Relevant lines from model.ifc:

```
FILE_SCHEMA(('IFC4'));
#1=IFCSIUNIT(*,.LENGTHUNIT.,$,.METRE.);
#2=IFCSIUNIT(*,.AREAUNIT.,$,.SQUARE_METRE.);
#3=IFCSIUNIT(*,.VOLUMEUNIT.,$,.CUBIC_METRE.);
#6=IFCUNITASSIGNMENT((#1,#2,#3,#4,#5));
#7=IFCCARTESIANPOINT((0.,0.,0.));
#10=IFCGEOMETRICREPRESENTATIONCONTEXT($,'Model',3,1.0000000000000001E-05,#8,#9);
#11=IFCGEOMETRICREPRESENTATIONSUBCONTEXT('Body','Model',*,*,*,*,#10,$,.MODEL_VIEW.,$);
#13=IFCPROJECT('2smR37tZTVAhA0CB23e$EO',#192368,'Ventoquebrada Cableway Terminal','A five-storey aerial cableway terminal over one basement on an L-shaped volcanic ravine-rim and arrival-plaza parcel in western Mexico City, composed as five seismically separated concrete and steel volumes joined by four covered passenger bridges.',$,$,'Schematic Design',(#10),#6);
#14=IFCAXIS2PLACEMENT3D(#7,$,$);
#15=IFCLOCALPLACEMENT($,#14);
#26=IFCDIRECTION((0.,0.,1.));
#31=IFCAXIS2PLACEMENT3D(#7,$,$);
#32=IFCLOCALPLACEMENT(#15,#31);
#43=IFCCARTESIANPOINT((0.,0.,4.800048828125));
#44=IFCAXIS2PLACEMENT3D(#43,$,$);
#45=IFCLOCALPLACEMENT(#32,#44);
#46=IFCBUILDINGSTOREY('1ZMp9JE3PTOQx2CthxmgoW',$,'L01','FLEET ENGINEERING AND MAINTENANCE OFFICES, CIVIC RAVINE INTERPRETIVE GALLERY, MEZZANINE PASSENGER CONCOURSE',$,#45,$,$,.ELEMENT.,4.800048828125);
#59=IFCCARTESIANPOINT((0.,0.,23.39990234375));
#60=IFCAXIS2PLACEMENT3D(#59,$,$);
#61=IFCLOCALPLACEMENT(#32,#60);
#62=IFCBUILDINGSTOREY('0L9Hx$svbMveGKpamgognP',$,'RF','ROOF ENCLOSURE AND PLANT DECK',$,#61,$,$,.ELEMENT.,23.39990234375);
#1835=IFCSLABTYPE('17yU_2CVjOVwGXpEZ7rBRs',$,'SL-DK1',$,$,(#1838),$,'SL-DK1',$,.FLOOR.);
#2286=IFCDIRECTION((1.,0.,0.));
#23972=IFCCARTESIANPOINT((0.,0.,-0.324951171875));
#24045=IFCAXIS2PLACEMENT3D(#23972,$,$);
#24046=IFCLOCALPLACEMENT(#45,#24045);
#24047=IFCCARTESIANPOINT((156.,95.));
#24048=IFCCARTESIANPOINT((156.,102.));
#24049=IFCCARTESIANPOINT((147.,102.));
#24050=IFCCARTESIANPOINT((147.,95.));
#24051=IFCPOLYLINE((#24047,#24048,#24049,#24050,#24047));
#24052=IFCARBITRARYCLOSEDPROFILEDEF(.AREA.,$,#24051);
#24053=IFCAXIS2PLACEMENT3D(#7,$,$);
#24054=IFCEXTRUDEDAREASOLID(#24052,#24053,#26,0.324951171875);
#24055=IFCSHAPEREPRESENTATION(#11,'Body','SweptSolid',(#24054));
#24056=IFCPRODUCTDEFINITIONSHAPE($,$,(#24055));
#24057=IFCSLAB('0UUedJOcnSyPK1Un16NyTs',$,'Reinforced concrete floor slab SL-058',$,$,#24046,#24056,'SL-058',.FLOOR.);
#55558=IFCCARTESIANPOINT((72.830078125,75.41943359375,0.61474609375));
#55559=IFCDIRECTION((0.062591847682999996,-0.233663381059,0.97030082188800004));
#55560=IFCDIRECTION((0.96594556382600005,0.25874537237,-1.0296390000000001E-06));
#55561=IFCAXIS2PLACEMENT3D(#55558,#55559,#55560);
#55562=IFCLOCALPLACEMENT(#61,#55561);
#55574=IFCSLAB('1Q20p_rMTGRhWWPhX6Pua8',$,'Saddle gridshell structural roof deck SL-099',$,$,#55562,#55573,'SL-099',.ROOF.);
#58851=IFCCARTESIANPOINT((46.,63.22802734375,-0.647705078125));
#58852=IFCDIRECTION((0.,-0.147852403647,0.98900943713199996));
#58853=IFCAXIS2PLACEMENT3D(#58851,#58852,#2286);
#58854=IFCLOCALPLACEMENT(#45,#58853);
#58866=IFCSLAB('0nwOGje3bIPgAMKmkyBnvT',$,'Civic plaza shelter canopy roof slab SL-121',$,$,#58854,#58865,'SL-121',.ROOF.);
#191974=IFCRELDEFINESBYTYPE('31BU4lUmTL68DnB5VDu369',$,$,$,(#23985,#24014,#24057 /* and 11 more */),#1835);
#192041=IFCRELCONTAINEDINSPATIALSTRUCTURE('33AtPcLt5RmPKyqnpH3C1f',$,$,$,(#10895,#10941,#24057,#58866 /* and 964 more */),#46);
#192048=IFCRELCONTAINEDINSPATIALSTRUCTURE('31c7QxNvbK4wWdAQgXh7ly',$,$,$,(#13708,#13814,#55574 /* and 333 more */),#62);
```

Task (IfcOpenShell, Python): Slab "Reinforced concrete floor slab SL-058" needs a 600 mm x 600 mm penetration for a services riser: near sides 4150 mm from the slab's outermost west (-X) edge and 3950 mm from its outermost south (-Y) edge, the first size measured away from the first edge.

```python
import numpy as np
import ifcopenshell
import ifcopenshell.api.feature
import ifcopenshell.api.geometry
import ifcopenshell.api.root
import ifcopenshell.geom
import ifcopenshell.util.placement
import ifcopenshell.util.representation
import ifcopenshell.util.shape
import ifcopenshell.util.unit

model = ifcopenshell.open("model.ifc")
unit_scale = ifcopenshell.util.unit.calculate_unit_scale(model)
settings = ifcopenshell.geom.settings()


def volume(element):
    """Net volume in cubic metres, openings subtracted."""
    shape = ifcopenshell.geom.create_shape(settings, element)
    return ifcopenshell.util.shape.get_volume(shape.geometry)


slab = model.by_id(24057)
before = volume(slab)

# Extent in the slab's own axes, in metres. The edges named are its -X and -Y sides.
slab_shape = ifcopenshell.geom.create_shape(settings, slab)
vertices = ifcopenshell.util.shape.get_vertices(slab_shape.geometry)
x_min, y_min, bottom = vertices.min(axis=0)
top = vertices[:, 2].max()

opening = ifcopenshell.api.root.create_entity(model, ifc_class="IfcOpeningElement", name="Services riser opening", predefined_type="OPENING")
context = ifcopenshell.util.representation.get_context(model, "Model", "Body", "MODEL_VIEW")
width, depth = 0.6, 0.6
outline = [(0.0, 0.0), (width, 0.0), (width, depth), (0.0, depth), (0.0, 0.0)]
# Overshoot both faces by 50 mm so the cut is clean.
shape = ifcopenshell.api.geometry.add_slab_representation(
    model, context=context, depth=top - bottom + 0.1, polyline=outline
)
ifcopenshell.api.geometry.assign_representation(model, product=opening, representation=shape)

matrix = ifcopenshell.util.placement.get_local_placement(slab.ObjectPlacement)
matrix[:, 3] = matrix @ np.append(np.array([x_min + 4.15, y_min + 3.95, bottom - 0.05]) / unit_scale, 1.0)
ifcopenshell.api.geometry.edit_object_placement(model, product=opening, matrix=matrix, is_si=False)
ifcopenshell.api.feature.add_feature(model, feature=opening, element=slab)

after = volume(slab)

print(f"slab volume {before:.3f} -> {after:.3f} m3")

model.write("model-out.ifc")
```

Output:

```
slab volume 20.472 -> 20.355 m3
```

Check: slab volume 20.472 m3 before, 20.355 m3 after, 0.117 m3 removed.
